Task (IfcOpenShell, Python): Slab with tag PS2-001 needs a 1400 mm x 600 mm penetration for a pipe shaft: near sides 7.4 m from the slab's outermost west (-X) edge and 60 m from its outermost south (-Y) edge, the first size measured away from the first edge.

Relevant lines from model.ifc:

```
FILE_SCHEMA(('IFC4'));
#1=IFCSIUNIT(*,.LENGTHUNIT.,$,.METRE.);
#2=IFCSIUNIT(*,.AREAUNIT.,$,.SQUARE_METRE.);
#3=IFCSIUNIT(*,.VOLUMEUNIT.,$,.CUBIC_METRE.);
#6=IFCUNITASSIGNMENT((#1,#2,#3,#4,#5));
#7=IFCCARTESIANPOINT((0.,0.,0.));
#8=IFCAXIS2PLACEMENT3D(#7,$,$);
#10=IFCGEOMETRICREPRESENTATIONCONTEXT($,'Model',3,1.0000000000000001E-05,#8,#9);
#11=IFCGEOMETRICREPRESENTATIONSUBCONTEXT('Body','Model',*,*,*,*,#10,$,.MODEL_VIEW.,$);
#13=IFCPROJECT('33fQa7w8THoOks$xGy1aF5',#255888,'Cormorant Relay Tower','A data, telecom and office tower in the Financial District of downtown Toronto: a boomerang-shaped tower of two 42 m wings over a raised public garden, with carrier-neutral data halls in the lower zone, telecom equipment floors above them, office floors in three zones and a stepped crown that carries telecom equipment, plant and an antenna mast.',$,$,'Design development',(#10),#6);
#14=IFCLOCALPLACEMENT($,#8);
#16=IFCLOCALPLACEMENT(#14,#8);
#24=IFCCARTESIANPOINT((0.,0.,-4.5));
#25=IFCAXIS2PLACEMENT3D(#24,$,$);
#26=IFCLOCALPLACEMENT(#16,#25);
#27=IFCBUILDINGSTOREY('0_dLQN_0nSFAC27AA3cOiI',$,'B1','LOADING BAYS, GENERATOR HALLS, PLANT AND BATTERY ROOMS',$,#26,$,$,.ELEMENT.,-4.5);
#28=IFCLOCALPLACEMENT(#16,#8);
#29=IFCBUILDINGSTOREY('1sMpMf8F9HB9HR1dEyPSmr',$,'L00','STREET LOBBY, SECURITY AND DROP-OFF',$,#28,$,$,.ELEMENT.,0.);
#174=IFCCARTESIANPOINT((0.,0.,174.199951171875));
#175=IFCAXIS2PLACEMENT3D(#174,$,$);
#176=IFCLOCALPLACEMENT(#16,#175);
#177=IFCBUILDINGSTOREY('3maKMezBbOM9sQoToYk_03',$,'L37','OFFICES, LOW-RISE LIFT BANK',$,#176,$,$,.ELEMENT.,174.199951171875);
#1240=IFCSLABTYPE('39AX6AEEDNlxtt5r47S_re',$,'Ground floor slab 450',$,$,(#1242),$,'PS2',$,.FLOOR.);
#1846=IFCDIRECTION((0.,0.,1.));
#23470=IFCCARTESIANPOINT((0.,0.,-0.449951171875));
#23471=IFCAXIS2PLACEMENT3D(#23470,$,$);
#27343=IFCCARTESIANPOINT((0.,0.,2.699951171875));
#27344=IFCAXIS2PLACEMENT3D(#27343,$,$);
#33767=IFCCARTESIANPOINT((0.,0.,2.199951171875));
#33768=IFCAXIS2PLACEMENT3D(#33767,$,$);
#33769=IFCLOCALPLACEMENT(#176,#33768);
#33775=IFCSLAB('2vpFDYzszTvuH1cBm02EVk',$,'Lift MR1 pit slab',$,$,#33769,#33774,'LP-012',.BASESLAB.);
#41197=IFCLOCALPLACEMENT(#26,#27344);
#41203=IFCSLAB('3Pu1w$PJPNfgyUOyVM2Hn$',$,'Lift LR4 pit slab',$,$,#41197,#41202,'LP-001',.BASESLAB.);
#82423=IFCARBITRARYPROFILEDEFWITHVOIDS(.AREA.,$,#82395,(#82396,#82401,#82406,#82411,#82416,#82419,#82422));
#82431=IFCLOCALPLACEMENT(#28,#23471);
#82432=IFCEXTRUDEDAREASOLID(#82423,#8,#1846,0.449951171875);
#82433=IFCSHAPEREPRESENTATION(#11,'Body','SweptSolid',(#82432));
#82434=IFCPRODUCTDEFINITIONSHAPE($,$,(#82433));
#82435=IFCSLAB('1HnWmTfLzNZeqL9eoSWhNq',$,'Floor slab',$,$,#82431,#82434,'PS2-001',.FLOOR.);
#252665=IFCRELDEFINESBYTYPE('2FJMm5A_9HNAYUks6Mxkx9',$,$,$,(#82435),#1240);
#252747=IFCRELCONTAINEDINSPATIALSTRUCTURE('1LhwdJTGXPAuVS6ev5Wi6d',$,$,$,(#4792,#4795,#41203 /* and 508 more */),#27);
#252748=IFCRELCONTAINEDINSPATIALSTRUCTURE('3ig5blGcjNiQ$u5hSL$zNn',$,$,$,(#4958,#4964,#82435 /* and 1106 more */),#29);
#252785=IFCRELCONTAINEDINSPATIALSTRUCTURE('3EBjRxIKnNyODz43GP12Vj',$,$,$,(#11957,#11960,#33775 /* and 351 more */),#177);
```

```python
import numpy as np
import ifcopenshell
import ifcopenshell.api.feature
import ifcopenshell.api.geometry
import ifcopenshell.api.root
import ifcopenshell.geom
import ifcopenshell.util.placement
import ifcopenshell.util.representation
import ifcopenshell.util.shape
import ifcopenshell.util.unit

model = ifcopenshell.open("model.ifc")
unit_scale = ifcopenshell.util.unit.calculate_unit_scale(model)
settings = ifcopenshell.geom.settings()


def volume(element):
    """Net volume in cubic metres, openings subtracted."""
    shape = ifcopenshell.geom.create_shape(settings, element)
    return ifcopenshell.util.shape.get_volume(shape.geometry)


slab = model.by_guid("1HnWmTfLzNZeqL9eoSWhNq")
before = volume(slab)

# Extent in the slab's own axes, in metres. The edges named are its -X and -Y sides.
slab_shape = ifcopenshell.geom.create_shape(settings, slab)
vertices = ifcopenshell.util.shape.get_vertices(slab_shape.geometry)
x_min, y_min, bottom = vertices.min(axis=0)
top = vertices[:, 2].max()

opening = ifcopenshell.api.root.create_entity(model, ifc_class="IfcOpeningElement", name="Pipe shaft opening", predefined_type="OPENING")
context = ifcopenshell.util.representation.get_context(model, "Model", "Body", "MODEL_VIEW")
width, depth = 1.4, 0.6
outline = [(0.0, 0.0), (width, 0.0), (width, depth), (0.0, depth), (0.0, 0.0)]
# Overshoot both faces by 50 mm so the cut is clean.
shape = ifcopenshell.api.geometry.add_slab_representation(
    model, context=context, depth=top - bottom + 0.1, polyline=outline
)
ifcopenshell.api.geometry.assign_representation(model, product=opening, representation=shape)

matrix = ifcopenshell.util.placement.get_local_placement(slab.ObjectPlacement)
matrix[:, 3] = matrix @ np.append(np.array([x_min + 7.4, y_min + 60, bottom - 0.05]) / unit_scale, 1.0)
ifcopenshell.api.geometry.edit_object_placement(model, product=opening, matrix=matrix, is_si=False)
ifcopenshell.api.feature.add_feature(model, feature=opening, element=slab)

after = volume(slab)

print(f"slab volume {before:.3f} -> {after:.3f} m3")

model.write("model_updated.ifc")
```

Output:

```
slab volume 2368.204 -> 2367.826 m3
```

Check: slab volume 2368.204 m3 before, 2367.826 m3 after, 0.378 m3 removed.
